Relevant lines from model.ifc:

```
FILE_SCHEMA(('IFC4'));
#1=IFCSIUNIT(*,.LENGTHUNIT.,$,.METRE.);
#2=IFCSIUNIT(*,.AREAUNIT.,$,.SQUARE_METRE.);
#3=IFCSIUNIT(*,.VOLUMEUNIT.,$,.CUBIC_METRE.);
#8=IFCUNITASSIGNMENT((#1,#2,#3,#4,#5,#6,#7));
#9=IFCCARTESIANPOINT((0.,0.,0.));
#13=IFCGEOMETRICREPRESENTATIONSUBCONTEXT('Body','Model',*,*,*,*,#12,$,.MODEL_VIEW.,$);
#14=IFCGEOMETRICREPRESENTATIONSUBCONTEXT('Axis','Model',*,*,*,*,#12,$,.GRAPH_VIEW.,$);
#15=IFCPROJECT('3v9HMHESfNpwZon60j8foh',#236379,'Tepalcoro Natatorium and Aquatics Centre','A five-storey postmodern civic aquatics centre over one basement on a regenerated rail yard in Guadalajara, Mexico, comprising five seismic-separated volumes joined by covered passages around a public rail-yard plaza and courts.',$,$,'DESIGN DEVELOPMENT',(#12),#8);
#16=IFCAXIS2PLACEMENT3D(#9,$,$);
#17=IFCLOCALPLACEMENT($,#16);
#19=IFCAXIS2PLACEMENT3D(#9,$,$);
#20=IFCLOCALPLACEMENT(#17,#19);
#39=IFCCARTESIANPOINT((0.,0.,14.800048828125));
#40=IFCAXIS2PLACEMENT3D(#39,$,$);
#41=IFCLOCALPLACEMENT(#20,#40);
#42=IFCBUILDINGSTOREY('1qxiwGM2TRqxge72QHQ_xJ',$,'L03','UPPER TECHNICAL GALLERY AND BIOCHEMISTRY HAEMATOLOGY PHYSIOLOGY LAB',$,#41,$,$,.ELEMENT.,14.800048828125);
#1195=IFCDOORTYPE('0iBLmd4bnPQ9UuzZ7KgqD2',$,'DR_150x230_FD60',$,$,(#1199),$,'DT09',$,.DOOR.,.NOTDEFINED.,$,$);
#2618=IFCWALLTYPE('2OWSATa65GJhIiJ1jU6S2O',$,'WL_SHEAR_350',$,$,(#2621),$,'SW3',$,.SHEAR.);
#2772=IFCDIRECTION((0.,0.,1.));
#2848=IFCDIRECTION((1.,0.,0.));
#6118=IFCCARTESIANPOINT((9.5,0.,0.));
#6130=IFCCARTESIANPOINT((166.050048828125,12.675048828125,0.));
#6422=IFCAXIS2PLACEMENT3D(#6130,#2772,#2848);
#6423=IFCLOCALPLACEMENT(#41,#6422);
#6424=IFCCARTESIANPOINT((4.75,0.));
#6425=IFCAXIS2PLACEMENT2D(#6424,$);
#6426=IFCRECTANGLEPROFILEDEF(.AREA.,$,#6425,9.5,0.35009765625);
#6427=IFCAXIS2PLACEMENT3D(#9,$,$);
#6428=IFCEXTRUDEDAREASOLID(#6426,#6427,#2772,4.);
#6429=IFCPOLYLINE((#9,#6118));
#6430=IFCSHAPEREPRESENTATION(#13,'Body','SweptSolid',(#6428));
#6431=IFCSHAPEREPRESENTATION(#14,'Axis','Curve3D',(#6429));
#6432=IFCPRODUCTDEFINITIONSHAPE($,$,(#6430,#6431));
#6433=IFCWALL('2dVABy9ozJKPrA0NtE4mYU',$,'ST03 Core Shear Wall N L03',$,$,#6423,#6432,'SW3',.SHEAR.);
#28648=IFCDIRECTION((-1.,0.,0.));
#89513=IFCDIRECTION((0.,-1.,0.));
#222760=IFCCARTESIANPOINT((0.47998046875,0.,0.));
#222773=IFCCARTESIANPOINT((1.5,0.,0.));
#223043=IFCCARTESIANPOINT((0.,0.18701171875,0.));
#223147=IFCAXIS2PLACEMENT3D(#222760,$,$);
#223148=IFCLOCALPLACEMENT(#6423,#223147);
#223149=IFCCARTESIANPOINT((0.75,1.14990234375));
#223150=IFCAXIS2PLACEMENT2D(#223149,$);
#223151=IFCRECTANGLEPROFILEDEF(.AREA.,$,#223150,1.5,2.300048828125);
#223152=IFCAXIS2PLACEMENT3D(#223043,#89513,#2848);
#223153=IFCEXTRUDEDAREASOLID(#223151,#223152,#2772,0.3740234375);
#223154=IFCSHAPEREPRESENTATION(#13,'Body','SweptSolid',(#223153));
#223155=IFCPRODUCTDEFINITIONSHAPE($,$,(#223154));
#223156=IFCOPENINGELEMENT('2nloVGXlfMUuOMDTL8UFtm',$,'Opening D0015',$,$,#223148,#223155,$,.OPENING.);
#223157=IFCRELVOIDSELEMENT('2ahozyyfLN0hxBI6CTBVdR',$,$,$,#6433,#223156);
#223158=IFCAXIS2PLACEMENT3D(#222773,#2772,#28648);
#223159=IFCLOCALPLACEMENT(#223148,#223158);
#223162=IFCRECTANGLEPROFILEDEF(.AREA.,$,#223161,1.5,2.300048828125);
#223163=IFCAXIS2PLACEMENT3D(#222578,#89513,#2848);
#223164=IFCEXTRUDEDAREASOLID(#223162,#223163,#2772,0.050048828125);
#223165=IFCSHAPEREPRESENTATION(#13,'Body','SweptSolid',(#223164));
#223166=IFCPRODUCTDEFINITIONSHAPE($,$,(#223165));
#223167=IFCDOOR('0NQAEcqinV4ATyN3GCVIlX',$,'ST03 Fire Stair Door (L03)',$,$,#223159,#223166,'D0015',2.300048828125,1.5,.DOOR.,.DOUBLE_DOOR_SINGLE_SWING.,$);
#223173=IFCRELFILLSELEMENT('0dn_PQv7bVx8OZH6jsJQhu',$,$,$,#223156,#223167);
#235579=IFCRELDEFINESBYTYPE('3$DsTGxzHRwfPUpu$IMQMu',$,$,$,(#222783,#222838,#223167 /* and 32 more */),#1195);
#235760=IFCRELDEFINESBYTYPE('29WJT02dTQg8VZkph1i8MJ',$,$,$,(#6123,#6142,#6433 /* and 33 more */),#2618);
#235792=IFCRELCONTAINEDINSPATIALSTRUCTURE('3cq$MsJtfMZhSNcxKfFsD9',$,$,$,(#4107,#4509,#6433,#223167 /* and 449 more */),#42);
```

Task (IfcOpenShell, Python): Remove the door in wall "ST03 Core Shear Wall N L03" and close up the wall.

```python
import ifcopenshell
import ifcopenshell.api.feature
import ifcopenshell.api.root
import ifcopenshell.geom
import ifcopenshell.util.shape

model = ifcopenshell.open("model.ifc")
settings = ifcopenshell.geom.settings()


def volume(element):
    """Net volume in cubic metres, openings subtracted."""
    shape = ifcopenshell.geom.create_shape(settings, element)
    return ifcopenshell.util.shape.get_volume(shape.geometry)


door = model.by_guid("0NQAEcqinV4ATyN3GCVIlX")
opening = door.FillsVoids[0].RelatingOpeningElement
wall = opening.VoidsElements[0].RelatingBuildingElement
before = volume(wall)

ifcopenshell.api.root.remove_product(model, product=door)
ifcopenshell.api.feature.remove_feature(model, feature=opening)

after = volume(wall)

print(f"wall volume {before:.3f} -> {after:.3f} m3")

model.write("model-out.ifc")
```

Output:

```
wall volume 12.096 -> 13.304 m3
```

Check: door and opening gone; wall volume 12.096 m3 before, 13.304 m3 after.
